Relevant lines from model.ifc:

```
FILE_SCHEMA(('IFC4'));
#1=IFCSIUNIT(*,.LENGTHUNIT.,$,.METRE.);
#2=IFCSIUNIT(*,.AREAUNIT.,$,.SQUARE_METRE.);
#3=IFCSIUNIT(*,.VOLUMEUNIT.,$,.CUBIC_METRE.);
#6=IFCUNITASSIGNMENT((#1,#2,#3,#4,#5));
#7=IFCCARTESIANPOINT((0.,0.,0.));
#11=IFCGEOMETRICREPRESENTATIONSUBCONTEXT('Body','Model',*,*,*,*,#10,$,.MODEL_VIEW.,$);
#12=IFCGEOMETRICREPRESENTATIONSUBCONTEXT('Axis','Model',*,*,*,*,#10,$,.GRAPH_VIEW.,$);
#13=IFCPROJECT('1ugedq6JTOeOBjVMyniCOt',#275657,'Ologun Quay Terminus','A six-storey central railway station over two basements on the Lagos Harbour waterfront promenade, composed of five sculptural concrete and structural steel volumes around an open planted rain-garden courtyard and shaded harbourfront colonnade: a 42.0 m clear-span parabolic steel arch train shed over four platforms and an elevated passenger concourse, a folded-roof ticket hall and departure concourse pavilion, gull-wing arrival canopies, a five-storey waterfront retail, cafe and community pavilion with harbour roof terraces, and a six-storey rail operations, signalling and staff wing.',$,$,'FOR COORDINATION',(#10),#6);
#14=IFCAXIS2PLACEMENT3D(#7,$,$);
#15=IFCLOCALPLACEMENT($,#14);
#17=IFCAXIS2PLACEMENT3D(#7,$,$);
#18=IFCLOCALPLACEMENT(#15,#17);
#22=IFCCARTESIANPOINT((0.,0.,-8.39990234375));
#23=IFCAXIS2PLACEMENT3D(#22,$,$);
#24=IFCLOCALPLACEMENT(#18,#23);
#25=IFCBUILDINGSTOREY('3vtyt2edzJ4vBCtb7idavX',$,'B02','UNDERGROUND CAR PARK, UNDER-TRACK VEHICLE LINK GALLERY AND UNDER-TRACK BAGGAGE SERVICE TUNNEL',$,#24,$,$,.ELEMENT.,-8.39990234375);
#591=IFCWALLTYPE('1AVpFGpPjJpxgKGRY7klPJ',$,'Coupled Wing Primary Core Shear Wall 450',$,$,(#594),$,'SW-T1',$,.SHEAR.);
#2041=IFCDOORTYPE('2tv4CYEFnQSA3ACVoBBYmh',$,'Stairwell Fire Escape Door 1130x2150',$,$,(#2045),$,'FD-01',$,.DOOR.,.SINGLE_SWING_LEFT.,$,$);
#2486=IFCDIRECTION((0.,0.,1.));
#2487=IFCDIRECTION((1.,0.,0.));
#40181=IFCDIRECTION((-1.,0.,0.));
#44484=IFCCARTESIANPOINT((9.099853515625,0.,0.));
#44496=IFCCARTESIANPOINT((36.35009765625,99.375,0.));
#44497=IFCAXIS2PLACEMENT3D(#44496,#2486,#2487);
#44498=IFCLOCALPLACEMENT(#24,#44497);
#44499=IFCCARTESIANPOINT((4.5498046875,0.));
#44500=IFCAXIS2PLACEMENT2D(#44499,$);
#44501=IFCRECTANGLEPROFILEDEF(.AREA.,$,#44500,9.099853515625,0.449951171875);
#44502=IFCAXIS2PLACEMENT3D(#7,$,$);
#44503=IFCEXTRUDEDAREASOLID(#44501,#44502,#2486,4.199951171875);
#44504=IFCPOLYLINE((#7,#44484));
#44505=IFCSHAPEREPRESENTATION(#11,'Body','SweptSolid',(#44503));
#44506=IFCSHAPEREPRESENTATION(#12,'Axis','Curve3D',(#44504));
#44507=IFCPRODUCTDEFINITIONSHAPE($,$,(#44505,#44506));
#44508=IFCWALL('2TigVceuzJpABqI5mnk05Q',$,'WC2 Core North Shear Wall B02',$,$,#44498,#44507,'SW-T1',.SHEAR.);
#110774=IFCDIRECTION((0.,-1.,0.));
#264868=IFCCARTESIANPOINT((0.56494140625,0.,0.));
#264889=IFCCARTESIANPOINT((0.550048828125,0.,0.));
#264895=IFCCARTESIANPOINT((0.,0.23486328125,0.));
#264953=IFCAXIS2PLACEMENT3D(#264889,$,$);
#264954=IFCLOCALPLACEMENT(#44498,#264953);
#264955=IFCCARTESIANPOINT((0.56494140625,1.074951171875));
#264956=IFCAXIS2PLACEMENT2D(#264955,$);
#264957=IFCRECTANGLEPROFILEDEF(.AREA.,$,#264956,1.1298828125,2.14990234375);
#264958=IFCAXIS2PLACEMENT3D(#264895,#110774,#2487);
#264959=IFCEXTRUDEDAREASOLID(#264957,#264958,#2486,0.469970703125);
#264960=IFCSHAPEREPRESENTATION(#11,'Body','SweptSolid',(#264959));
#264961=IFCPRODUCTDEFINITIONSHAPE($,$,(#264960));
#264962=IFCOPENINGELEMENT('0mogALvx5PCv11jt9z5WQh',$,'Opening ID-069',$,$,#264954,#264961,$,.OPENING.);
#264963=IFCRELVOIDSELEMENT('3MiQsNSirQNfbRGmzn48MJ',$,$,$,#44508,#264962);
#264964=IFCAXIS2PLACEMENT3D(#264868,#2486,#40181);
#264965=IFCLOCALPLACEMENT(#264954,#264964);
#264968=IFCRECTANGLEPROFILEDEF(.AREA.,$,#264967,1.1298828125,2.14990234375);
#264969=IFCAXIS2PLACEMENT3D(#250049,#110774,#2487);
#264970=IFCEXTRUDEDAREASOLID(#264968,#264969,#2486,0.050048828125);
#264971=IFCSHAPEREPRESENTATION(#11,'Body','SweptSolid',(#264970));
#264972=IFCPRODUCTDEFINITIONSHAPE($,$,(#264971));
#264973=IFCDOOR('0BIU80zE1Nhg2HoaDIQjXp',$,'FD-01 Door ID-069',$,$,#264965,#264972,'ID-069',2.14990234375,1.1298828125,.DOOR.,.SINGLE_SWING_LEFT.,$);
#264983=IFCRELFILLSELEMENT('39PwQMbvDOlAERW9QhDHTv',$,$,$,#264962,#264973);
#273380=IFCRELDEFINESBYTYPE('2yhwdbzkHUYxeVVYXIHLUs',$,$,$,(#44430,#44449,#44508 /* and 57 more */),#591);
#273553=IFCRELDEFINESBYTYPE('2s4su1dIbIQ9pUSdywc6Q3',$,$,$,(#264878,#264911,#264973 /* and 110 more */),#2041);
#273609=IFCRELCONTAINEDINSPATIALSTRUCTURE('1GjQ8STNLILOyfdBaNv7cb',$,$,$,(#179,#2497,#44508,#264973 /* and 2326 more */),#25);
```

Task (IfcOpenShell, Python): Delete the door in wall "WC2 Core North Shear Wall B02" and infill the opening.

```python
import ifcopenshell
import ifcopenshell.api.feature
import ifcopenshell.api.root
import ifcopenshell.geom
import ifcopenshell.util.shape

model = ifcopenshell.open("model.ifc")
settings = ifcopenshell.geom.settings()


def volume(element):
    """Net volume in cubic metres, openings subtracted."""
    shape = ifcopenshell.geom.create_shape(settings, element)
    return ifcopenshell.util.shape.get_volume(shape.geometry)


door = model.by_id(264973)
opening = door.FillsVoids[0].RelatingOpeningElement
wall = opening.VoidsElements[0].RelatingBuildingElement
before = volume(wall)

ifcopenshell.api.root.remove_product(model, product=door)
ifcopenshell.api.feature.remove_feature(model, feature=opening)

after = volume(wall)

print(f"wall volume {before:.3f} -> {after:.3f} m3")

model.write("model_edited.ifc")
```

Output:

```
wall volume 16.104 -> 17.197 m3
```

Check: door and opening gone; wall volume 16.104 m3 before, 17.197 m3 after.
